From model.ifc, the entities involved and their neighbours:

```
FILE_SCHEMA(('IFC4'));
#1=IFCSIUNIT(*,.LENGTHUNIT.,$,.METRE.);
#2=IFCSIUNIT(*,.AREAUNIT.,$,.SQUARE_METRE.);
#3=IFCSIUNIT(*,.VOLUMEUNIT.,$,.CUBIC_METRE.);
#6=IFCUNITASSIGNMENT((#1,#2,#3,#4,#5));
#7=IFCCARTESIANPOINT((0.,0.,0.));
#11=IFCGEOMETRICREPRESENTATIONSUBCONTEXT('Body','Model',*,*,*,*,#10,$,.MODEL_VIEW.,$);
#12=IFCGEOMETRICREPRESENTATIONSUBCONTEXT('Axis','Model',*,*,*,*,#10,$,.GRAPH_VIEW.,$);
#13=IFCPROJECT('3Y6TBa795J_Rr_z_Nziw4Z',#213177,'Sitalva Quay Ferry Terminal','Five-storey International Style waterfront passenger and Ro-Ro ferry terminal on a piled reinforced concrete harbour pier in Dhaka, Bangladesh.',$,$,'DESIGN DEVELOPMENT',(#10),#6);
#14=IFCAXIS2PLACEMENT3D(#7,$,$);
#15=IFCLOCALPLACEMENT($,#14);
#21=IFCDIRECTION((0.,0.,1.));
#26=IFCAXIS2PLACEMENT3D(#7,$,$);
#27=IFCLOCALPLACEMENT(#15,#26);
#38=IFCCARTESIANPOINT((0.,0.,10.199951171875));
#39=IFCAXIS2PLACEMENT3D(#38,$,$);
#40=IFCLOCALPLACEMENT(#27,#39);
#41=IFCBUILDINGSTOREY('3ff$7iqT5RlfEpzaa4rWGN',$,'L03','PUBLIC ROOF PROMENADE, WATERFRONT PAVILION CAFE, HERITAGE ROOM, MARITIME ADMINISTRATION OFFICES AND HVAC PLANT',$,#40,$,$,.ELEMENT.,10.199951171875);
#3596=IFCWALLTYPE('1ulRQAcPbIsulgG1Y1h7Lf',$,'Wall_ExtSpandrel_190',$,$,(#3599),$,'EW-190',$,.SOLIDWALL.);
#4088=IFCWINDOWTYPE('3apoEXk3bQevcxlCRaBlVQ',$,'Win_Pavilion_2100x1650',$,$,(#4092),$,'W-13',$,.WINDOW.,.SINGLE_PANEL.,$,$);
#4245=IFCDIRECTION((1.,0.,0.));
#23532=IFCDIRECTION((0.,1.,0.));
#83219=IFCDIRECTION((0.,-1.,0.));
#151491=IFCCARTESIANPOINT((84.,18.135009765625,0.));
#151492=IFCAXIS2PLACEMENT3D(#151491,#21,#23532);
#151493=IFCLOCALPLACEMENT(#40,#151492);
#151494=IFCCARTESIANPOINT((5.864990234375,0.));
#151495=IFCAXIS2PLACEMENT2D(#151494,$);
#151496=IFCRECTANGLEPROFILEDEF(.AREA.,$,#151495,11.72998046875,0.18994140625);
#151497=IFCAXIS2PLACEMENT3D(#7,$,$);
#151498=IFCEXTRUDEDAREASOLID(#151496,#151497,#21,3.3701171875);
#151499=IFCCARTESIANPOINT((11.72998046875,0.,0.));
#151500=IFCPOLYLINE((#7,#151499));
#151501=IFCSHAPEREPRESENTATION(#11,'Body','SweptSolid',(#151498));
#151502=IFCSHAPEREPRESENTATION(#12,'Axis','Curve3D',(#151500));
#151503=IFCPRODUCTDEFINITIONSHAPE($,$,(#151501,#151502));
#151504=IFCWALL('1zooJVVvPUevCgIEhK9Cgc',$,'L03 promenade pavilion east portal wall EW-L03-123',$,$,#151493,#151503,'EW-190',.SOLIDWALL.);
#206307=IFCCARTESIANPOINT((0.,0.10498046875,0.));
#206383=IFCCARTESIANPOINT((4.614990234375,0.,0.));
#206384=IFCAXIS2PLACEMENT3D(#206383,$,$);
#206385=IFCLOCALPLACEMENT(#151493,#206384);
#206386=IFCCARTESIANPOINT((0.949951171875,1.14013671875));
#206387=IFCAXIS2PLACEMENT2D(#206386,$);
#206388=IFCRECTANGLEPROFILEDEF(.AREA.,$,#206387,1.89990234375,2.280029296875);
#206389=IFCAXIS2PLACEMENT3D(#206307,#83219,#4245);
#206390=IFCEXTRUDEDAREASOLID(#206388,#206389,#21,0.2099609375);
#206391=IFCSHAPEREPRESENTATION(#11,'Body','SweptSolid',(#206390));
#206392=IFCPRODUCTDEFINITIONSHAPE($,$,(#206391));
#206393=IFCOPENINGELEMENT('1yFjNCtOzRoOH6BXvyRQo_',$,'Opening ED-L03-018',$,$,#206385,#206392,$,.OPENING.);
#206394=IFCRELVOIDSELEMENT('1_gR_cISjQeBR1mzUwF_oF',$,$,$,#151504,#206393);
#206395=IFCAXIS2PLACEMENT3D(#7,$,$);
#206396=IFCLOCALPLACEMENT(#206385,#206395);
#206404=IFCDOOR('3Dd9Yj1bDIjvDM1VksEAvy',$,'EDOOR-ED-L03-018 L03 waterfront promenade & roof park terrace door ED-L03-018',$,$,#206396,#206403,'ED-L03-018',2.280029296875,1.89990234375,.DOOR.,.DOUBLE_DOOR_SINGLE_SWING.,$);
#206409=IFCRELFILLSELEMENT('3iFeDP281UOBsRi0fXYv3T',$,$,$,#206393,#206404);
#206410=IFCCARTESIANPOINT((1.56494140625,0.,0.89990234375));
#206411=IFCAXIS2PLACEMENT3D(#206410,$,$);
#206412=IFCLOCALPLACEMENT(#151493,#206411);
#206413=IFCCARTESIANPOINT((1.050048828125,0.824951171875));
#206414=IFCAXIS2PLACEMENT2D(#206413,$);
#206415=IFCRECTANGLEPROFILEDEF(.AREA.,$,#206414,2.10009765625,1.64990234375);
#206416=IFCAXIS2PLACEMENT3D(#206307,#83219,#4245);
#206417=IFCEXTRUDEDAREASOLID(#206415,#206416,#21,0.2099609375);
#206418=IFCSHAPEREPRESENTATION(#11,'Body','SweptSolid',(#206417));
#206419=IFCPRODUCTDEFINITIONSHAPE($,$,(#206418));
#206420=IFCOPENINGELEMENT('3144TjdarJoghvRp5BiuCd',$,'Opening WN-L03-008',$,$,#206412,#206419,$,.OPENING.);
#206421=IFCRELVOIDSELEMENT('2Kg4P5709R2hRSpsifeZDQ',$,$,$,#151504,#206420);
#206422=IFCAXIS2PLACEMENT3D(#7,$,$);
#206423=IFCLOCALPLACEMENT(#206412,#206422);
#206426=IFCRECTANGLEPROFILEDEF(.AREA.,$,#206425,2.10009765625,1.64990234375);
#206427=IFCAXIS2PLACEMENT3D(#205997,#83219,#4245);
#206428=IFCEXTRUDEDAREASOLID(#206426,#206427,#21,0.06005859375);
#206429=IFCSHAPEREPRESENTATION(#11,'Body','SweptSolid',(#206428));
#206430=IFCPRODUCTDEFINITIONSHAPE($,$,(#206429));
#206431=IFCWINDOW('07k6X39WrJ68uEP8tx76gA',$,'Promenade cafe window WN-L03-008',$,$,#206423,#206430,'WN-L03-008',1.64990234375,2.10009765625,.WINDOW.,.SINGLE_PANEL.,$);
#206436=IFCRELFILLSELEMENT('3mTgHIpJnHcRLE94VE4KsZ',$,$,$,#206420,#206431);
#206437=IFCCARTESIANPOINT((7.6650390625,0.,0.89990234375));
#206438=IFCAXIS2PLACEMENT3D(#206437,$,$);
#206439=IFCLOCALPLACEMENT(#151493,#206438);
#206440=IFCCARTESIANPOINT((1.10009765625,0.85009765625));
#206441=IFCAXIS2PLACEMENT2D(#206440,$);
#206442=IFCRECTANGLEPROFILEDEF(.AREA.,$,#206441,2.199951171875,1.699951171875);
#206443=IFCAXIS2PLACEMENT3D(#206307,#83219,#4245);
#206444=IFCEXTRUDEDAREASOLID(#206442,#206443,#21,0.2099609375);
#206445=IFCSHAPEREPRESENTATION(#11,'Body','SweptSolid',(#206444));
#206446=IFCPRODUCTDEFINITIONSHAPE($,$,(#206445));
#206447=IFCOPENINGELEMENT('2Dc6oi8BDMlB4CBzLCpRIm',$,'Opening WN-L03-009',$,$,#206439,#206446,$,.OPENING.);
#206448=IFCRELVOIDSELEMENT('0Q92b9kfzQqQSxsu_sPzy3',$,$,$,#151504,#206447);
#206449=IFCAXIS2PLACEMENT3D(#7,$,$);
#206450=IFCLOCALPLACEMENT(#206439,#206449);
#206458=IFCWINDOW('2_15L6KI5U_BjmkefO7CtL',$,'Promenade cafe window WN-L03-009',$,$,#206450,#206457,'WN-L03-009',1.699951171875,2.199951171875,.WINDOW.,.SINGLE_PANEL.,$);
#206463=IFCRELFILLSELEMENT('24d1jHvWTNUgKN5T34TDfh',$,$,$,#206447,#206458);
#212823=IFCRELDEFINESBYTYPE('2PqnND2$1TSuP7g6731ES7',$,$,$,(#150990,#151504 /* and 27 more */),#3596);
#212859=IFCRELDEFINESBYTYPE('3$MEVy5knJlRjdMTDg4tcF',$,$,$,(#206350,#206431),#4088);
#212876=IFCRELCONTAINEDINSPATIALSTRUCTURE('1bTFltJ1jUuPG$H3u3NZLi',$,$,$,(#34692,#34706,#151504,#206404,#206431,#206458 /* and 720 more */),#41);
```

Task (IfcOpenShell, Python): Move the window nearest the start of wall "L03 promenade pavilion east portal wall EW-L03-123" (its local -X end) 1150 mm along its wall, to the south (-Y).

```python
import ifcopenshell
import ifcopenshell.api.geometry
import ifcopenshell.util.placement
import ifcopenshell.util.unit

model = ifcopenshell.open("model.ifc")
unit_scale = ifcopenshell.util.unit.calculate_unit_scale(model)

window = model.by_guid("07k6X39WrJ68uEP8tx76gA")
opening = window.FillsVoids[0].RelatingOpeningElement
wall = opening.VoidsElements[0].RelatingBuildingElement

wall_matrix = ifcopenshell.util.placement.get_local_placement(wall.ObjectPlacement)
shift = wall_matrix[:3, 0] * -1.15 / unit_scale
before = ifcopenshell.util.placement.get_local_placement(window.ObjectPlacement)[:3, 3].copy()

# The window is placed relative to its opening, so it follows when the opening moves.
matrix = ifcopenshell.util.placement.get_local_placement(opening.ObjectPlacement)
matrix[:3, 3] += shift
ifcopenshell.api.geometry.edit_object_placement(
    model, product=opening, matrix=matrix, is_si=False, should_transform_children=True
)

after = ifcopenshell.util.placement.get_local_placement(window.ObjectPlacement)[:3, 3]
print("window moved by", (after - before).round(3) + 0.0)

model.write("model_updated.ifc")
```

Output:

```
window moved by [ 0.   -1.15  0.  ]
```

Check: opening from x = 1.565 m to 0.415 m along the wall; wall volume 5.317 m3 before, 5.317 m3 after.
